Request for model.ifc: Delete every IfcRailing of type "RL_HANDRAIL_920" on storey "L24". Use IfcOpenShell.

First a look at what the model holds.

```python
import ifcopenshell
import ifcopenshell.util.element

model = ifcopenshell.open("model.ifc")
print(model.schema)
storey = next(s for s in model.by_type("IfcBuildingStorey") if s.Name == "L24")
railings = [e for e in ifcopenshell.util.element.get_decomposition(storey) if e.is_a("IfcRailing")]
seen = {}
for e in railings:
    element_type = ifcopenshell.util.element.get_type(e)
    name = element_type.Name if element_type not in (None, e) else None
    seen[name] = seen.get(name, 0) + 1
for name, count in sorted(seen.items(), key=str):
    print(count, "x", name)
```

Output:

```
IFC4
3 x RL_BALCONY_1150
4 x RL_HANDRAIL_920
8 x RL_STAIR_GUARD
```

```python
import ifcopenshell
import ifcopenshell.api.root
import ifcopenshell.util.element

model = ifcopenshell.open("model.ifc")

storey = next(s for s in model.by_type("IfcBuildingStorey") if s.Name == "L24")
railings = [e for e in ifcopenshell.util.element.get_decomposition(storey) if e.is_a("IfcRailing")]
targets = [e for e in railings if (t := ifcopenshell.util.element.get_type(e)) not in (None, e) and t.Name == "RL_HANDRAIL_920"]

for e in targets:
    ifcopenshell.api.root.remove_product(model, product=e)
print(len(targets), "removed")

model.write("model_rev.ifc")
```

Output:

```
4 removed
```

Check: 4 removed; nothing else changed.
